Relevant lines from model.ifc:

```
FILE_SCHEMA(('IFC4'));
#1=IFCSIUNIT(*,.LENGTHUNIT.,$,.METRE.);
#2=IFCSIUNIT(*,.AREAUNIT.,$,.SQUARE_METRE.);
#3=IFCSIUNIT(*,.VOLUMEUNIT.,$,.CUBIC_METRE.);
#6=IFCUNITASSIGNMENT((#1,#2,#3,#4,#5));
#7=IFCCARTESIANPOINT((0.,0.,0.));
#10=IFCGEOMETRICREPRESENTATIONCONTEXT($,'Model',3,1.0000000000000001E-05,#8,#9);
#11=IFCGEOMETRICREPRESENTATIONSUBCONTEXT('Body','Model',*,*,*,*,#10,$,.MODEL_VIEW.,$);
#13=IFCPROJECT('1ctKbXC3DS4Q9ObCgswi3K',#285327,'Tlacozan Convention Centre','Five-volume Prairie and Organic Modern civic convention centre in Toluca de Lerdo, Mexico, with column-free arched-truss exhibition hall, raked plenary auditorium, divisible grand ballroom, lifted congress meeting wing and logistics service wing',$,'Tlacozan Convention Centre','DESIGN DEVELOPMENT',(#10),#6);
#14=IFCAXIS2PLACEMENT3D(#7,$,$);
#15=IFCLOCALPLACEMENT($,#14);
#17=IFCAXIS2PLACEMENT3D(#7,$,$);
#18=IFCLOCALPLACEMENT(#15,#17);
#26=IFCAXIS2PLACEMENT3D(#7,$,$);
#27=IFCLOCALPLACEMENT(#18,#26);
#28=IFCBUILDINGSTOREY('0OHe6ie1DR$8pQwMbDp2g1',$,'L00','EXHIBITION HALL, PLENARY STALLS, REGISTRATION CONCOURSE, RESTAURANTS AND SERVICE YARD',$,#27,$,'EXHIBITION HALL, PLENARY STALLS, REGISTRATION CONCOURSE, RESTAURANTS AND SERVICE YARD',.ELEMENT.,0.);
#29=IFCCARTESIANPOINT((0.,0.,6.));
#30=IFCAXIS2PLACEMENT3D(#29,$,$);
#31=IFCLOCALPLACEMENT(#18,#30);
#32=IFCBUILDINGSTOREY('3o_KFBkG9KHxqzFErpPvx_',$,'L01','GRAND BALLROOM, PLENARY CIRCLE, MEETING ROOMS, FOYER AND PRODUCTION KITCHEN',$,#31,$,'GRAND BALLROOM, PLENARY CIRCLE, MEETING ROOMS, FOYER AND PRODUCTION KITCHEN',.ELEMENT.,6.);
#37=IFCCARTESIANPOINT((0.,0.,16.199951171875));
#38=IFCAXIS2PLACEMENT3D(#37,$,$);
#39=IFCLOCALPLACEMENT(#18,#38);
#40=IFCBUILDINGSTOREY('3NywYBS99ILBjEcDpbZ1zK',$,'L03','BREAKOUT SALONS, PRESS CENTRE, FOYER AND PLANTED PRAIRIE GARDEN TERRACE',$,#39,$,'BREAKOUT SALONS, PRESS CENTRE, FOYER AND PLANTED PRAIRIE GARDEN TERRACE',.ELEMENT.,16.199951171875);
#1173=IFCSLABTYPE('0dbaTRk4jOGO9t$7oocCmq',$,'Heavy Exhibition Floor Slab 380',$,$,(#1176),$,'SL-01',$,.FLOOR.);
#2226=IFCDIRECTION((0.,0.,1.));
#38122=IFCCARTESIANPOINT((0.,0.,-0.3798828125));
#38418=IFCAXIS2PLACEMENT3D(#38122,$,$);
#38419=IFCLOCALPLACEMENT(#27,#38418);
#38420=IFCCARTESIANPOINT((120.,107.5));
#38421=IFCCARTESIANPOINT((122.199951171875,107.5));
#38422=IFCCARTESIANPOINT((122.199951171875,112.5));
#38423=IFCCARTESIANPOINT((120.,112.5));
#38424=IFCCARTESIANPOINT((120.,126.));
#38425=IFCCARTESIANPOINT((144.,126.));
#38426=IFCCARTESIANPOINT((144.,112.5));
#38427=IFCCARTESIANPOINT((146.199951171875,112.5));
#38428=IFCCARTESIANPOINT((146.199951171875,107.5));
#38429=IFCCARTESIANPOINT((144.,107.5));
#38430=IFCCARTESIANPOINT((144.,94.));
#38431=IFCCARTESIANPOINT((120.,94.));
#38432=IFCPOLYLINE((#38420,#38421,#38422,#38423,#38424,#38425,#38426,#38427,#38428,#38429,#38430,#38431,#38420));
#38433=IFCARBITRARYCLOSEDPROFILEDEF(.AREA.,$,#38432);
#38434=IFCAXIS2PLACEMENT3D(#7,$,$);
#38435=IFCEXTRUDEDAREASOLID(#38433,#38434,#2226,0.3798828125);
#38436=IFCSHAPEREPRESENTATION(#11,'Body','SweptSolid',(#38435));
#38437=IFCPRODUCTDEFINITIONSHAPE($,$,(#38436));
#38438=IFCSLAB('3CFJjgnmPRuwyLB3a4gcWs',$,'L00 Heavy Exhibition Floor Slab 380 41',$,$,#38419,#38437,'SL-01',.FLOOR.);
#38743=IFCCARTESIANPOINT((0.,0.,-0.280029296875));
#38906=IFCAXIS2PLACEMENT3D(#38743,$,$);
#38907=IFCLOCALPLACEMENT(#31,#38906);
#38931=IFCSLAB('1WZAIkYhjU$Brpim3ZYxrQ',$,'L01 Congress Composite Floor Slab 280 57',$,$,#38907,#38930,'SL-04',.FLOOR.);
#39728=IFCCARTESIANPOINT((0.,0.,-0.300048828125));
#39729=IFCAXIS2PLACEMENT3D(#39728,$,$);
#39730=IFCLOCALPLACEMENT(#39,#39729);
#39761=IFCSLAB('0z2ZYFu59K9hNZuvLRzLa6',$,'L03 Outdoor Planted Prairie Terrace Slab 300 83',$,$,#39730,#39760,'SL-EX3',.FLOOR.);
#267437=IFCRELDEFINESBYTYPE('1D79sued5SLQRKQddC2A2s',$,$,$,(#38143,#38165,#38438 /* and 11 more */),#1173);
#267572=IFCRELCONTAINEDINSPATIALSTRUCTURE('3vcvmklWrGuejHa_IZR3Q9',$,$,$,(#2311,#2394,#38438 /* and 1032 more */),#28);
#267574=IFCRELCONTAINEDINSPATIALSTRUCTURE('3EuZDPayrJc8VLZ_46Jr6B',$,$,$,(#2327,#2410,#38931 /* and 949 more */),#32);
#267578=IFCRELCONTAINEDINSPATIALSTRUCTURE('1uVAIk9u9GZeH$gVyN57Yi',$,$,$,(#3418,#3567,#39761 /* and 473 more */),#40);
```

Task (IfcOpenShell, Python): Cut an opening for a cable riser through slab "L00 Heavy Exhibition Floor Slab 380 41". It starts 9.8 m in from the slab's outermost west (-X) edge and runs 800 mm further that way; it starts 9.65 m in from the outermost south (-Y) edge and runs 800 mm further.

```python
import numpy as np
import ifcopenshell
import ifcopenshell.api.feature
import ifcopenshell.api.geometry
import ifcopenshell.api.root
import ifcopenshell.geom
import ifcopenshell.util.placement
import ifcopenshell.util.representation
import ifcopenshell.util.shape
import ifcopenshell.util.unit

model = ifcopenshell.open("model.ifc")
unit_scale = ifcopenshell.util.unit.calculate_unit_scale(model)
settings = ifcopenshell.geom.settings()


def volume(element):
    """Net volume in cubic metres, openings subtracted."""
    shape = ifcopenshell.geom.create_shape(settings, element)
    return ifcopenshell.util.shape.get_volume(shape.geometry)


slab = model.by_guid("3CFJjgnmPRuwyLB3a4gcWs")
before = volume(slab)

# Extent in the slab's own axes, in metres. The edges named are its -X and -Y sides.
slab_shape = ifcopenshell.geom.create_shape(settings, slab)
vertices = ifcopenshell.util.shape.get_vertices(slab_shape.geometry)
x_min, y_min, bottom = vertices.min(axis=0)
top = vertices[:, 2].max()

opening = ifcopenshell.api.root.create_entity(model, ifc_class="IfcOpeningElement", name="Cable riser opening", predefined_type="OPENING")
context = ifcopenshell.util.representation.get_context(model, "Model", "Body", "MODEL_VIEW")
width, depth = 0.8, 0.8
outline = [(0.0, 0.0), (width, 0.0), (width, depth), (0.0, depth), (0.0, 0.0)]
# Overshoot both faces by 50 mm so the cut is clean.
shape = ifcopenshell.api.geometry.add_slab_representation(
    model, context=context, depth=top - bottom + 0.1, polyline=outline
)
ifcopenshell.api.geometry.assign_representation(model, product=opening, representation=shape)

matrix = ifcopenshell.util.placement.get_local_placement(slab.ObjectPlacement)
matrix[:, 3] = matrix @ np.append(np.array([x_min + 9.8, y_min + 9.65, bottom - 0.05]) / unit_scale, 1.0)
ifcopenshell.api.geometry.edit_object_placement(model, product=opening, matrix=matrix, is_si=False)
ifcopenshell.api.feature.add_feature(model, feature=opening, element=slab)

after = volume(slab)

print(f"slab volume {before:.3f} -> {after:.3f} m3")

model.write("model_rev.ifc")
```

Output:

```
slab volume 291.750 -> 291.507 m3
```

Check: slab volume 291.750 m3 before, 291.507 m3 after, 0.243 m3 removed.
